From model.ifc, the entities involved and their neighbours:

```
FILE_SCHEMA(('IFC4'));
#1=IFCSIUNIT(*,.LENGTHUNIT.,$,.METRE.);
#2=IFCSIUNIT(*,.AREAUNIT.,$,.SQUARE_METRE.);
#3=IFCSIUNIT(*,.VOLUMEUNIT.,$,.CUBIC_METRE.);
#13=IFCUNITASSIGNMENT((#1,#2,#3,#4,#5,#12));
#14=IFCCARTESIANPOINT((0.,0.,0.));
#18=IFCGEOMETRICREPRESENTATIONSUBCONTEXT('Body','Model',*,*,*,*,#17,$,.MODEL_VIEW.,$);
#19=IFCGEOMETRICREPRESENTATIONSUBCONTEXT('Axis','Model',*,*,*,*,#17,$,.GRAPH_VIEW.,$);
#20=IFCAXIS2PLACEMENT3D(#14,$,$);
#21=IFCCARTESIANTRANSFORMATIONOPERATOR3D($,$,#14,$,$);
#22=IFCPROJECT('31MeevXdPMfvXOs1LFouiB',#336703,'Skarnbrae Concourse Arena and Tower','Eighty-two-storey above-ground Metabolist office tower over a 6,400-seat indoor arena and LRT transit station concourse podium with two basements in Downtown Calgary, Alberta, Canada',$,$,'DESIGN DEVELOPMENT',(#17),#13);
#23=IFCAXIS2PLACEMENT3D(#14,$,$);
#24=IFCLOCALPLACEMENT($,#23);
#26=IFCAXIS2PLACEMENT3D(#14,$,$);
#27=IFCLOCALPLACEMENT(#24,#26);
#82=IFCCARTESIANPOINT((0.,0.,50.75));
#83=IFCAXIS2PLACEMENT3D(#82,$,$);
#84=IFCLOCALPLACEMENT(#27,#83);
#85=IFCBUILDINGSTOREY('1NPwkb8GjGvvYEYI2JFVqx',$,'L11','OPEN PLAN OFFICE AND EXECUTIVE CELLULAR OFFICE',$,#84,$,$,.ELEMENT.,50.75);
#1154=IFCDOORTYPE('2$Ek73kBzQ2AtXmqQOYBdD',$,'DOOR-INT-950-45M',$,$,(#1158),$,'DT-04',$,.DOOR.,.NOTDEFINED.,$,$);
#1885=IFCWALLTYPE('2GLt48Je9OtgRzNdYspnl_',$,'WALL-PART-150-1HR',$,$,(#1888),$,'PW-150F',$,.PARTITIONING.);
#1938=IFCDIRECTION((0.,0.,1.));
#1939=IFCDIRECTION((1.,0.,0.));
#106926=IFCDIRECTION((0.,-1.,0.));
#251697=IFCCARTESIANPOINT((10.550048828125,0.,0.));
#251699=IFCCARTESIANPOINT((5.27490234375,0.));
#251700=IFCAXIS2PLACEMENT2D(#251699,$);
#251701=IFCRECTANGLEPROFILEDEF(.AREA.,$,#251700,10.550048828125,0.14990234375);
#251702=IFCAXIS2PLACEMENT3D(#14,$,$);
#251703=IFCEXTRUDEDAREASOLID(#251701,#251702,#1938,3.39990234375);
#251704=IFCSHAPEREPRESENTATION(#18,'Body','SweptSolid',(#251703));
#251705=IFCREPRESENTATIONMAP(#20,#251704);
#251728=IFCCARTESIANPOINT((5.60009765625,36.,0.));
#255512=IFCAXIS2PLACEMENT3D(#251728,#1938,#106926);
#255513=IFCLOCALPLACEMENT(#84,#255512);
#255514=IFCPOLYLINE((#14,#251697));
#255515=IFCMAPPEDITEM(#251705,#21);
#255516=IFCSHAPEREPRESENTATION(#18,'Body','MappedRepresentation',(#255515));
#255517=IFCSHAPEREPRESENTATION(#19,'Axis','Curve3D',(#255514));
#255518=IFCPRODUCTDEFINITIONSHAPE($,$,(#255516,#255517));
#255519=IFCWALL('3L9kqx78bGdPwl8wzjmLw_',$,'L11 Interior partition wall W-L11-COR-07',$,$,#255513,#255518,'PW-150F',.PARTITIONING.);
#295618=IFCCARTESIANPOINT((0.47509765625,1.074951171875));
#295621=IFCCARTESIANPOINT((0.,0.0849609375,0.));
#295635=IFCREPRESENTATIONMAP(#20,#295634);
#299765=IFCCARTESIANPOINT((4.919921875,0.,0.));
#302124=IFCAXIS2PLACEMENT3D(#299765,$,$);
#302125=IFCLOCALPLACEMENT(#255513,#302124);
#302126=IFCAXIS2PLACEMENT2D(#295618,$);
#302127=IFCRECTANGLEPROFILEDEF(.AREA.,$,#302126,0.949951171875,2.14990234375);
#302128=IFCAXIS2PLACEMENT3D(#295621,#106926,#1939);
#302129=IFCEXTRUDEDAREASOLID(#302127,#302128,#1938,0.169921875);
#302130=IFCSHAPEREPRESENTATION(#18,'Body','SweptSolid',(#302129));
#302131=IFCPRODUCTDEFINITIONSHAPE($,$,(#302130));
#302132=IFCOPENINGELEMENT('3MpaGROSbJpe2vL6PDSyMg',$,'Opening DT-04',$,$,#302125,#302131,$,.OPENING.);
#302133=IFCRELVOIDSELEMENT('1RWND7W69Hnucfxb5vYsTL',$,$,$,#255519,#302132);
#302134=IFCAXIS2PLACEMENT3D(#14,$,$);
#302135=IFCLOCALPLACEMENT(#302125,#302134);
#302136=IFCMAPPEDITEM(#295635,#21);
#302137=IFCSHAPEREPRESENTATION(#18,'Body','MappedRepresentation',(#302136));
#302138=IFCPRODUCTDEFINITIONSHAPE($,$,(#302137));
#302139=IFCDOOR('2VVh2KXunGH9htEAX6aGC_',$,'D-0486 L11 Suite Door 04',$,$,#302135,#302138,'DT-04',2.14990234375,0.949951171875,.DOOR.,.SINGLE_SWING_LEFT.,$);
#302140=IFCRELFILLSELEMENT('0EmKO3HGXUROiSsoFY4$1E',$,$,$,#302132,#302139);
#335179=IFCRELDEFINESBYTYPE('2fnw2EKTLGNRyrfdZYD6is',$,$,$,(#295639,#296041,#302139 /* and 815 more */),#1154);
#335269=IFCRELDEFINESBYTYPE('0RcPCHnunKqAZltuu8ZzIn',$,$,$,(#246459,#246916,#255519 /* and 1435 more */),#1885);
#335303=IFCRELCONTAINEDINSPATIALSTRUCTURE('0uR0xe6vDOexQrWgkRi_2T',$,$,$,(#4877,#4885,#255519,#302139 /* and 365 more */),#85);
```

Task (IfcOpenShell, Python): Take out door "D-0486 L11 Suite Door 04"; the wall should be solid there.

```python
import ifcopenshell
import ifcopenshell.api.feature
import ifcopenshell.api.root
import ifcopenshell.geom
import ifcopenshell.util.shape

model = ifcopenshell.open("model.ifc")
settings = ifcopenshell.geom.settings()


def volume(element):
    """Net volume in cubic metres, openings subtracted."""
    shape = ifcopenshell.geom.create_shape(settings, element)
    return ifcopenshell.util.shape.get_volume(shape.geometry)


door = model.by_guid("2VVh2KXunGH9htEAX6aGC_")
opening = door.FillsVoids[0].RelatingOpeningElement
wall = opening.VoidsElements[0].RelatingBuildingElement
before = volume(wall)

ifcopenshell.api.root.remove_product(model, product=door)
ifcopenshell.api.feature.remove_feature(model, feature=opening)

after = volume(wall)

print(f"wall volume {before:.3f} -> {after:.3f} m3")

model.write("model_rev.ifc")
```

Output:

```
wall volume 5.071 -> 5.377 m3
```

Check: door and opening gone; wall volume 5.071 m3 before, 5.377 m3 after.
